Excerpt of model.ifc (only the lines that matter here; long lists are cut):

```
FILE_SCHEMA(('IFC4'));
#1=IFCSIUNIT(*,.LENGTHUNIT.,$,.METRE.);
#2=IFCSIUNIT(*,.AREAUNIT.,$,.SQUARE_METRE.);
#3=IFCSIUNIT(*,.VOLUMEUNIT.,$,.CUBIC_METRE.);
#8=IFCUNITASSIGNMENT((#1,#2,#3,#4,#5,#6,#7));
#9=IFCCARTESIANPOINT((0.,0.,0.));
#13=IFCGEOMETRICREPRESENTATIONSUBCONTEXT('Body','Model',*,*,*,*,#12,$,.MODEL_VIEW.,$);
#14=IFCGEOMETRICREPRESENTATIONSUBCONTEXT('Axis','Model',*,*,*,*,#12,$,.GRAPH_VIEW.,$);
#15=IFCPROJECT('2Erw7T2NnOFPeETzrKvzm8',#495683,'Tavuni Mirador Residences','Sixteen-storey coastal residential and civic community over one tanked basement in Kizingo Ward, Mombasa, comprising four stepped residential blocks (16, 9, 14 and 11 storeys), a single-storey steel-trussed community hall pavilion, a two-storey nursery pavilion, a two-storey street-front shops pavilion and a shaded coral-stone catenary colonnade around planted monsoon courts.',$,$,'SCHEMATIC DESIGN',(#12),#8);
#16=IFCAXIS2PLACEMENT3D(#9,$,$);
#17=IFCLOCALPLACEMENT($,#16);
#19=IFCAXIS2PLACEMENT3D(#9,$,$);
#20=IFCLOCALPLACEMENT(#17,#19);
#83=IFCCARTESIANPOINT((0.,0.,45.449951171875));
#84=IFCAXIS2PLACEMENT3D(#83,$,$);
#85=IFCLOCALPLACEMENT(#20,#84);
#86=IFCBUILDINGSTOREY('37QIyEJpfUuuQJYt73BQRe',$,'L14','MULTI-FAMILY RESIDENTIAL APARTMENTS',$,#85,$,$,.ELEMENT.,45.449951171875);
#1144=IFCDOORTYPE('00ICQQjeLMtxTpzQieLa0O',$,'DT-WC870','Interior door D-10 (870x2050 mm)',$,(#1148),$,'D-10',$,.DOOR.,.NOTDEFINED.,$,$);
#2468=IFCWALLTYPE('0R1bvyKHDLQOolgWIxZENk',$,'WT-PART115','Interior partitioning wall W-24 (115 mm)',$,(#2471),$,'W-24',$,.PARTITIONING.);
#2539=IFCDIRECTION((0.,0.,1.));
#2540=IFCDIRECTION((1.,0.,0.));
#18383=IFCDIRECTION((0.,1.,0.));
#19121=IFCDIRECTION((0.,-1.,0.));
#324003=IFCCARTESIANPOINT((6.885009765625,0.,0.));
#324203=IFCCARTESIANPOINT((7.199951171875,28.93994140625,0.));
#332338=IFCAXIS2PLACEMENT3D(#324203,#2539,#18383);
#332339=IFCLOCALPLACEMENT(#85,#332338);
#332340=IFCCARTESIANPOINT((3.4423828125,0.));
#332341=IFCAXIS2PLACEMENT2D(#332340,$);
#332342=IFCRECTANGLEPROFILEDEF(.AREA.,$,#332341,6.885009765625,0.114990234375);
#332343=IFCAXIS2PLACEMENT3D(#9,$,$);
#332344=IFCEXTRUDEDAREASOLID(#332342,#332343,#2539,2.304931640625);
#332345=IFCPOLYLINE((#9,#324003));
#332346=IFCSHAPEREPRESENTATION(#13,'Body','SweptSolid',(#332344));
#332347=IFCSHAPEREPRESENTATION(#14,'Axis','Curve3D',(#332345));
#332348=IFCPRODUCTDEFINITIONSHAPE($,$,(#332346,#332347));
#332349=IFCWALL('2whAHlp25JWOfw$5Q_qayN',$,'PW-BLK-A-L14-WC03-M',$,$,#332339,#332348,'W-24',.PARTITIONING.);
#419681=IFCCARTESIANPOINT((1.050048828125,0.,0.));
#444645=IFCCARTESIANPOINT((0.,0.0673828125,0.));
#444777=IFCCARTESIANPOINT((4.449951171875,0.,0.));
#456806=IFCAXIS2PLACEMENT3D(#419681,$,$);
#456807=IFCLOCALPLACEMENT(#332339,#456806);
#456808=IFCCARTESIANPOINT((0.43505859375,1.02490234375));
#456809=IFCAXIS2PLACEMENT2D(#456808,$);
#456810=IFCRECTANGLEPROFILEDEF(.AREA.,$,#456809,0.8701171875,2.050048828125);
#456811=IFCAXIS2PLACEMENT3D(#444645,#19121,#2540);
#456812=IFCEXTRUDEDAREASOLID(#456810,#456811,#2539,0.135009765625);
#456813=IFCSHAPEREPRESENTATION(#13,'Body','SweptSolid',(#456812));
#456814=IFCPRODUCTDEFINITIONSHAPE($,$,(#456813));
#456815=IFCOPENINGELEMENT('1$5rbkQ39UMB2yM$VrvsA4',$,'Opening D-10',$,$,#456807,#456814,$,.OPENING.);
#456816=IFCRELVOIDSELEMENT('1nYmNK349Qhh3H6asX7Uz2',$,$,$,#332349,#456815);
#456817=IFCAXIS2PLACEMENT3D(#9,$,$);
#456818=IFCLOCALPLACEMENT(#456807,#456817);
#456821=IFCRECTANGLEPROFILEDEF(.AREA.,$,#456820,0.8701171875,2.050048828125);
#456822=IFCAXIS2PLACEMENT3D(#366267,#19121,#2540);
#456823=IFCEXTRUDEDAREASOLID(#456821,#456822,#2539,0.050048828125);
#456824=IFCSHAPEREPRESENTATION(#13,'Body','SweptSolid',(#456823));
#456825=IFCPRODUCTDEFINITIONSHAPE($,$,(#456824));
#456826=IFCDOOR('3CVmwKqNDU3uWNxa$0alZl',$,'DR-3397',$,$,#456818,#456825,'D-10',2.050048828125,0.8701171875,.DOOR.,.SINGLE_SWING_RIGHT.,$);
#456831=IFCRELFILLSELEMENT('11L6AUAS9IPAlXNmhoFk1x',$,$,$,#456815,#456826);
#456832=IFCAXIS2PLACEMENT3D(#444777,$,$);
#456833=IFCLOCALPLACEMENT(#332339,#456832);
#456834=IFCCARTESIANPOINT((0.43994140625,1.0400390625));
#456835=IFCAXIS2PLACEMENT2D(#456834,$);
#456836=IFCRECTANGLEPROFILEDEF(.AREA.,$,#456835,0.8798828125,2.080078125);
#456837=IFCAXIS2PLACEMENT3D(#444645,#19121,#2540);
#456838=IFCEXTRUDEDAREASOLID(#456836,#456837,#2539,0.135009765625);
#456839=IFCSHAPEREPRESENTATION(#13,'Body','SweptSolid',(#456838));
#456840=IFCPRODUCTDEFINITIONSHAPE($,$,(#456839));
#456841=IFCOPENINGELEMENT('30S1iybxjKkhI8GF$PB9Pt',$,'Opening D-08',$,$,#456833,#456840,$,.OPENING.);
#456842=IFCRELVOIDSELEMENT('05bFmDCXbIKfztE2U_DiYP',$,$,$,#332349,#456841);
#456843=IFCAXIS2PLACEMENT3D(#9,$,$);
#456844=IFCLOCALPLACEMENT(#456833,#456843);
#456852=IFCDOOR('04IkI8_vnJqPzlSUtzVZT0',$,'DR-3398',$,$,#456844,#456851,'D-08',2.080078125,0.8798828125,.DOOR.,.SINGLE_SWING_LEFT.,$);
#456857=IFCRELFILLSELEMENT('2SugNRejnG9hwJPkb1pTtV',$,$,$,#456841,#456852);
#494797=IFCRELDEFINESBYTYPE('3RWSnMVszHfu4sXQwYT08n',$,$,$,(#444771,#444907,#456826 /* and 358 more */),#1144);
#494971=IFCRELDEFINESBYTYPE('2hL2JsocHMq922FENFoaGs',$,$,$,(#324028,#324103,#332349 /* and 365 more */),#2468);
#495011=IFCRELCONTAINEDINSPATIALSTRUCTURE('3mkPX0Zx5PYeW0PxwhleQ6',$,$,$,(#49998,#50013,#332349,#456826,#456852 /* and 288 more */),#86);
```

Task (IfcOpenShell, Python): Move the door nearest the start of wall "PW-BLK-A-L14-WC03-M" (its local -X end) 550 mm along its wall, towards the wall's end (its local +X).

```python
import ifcopenshell
import ifcopenshell.api.geometry
import ifcopenshell.util.placement

model = ifcopenshell.open("model.ifc")

door = model.by_guid("3CVmwKqNDU3uWNxa$0alZl")
opening = door.FillsVoids[0].RelatingOpeningElement
wall = opening.VoidsElements[0].RelatingBuildingElement

wall_matrix = ifcopenshell.util.placement.get_local_placement(wall.ObjectPlacement)
shift = wall_matrix[:3, 0] * 0.55
before = ifcopenshell.util.placement.get_local_placement(door.ObjectPlacement)[:3, 3].copy()

# The door is placed relative to its opening, so it follows when the opening moves.
matrix = ifcopenshell.util.placement.get_local_placement(opening.ObjectPlacement)
matrix[:3, 3] += shift
ifcopenshell.api.geometry.edit_object_placement(
    model, product=opening, matrix=matrix, is_si=False, should_transform_children=True
)

after = ifcopenshell.util.placement.get_local_placement(door.ObjectPlacement)[:3, 3]
print("door moved by", (after - before).round(3) + 0.0)

model.write("model_updated.ifc")
```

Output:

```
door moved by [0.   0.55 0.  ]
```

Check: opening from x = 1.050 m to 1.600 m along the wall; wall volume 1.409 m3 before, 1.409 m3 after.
